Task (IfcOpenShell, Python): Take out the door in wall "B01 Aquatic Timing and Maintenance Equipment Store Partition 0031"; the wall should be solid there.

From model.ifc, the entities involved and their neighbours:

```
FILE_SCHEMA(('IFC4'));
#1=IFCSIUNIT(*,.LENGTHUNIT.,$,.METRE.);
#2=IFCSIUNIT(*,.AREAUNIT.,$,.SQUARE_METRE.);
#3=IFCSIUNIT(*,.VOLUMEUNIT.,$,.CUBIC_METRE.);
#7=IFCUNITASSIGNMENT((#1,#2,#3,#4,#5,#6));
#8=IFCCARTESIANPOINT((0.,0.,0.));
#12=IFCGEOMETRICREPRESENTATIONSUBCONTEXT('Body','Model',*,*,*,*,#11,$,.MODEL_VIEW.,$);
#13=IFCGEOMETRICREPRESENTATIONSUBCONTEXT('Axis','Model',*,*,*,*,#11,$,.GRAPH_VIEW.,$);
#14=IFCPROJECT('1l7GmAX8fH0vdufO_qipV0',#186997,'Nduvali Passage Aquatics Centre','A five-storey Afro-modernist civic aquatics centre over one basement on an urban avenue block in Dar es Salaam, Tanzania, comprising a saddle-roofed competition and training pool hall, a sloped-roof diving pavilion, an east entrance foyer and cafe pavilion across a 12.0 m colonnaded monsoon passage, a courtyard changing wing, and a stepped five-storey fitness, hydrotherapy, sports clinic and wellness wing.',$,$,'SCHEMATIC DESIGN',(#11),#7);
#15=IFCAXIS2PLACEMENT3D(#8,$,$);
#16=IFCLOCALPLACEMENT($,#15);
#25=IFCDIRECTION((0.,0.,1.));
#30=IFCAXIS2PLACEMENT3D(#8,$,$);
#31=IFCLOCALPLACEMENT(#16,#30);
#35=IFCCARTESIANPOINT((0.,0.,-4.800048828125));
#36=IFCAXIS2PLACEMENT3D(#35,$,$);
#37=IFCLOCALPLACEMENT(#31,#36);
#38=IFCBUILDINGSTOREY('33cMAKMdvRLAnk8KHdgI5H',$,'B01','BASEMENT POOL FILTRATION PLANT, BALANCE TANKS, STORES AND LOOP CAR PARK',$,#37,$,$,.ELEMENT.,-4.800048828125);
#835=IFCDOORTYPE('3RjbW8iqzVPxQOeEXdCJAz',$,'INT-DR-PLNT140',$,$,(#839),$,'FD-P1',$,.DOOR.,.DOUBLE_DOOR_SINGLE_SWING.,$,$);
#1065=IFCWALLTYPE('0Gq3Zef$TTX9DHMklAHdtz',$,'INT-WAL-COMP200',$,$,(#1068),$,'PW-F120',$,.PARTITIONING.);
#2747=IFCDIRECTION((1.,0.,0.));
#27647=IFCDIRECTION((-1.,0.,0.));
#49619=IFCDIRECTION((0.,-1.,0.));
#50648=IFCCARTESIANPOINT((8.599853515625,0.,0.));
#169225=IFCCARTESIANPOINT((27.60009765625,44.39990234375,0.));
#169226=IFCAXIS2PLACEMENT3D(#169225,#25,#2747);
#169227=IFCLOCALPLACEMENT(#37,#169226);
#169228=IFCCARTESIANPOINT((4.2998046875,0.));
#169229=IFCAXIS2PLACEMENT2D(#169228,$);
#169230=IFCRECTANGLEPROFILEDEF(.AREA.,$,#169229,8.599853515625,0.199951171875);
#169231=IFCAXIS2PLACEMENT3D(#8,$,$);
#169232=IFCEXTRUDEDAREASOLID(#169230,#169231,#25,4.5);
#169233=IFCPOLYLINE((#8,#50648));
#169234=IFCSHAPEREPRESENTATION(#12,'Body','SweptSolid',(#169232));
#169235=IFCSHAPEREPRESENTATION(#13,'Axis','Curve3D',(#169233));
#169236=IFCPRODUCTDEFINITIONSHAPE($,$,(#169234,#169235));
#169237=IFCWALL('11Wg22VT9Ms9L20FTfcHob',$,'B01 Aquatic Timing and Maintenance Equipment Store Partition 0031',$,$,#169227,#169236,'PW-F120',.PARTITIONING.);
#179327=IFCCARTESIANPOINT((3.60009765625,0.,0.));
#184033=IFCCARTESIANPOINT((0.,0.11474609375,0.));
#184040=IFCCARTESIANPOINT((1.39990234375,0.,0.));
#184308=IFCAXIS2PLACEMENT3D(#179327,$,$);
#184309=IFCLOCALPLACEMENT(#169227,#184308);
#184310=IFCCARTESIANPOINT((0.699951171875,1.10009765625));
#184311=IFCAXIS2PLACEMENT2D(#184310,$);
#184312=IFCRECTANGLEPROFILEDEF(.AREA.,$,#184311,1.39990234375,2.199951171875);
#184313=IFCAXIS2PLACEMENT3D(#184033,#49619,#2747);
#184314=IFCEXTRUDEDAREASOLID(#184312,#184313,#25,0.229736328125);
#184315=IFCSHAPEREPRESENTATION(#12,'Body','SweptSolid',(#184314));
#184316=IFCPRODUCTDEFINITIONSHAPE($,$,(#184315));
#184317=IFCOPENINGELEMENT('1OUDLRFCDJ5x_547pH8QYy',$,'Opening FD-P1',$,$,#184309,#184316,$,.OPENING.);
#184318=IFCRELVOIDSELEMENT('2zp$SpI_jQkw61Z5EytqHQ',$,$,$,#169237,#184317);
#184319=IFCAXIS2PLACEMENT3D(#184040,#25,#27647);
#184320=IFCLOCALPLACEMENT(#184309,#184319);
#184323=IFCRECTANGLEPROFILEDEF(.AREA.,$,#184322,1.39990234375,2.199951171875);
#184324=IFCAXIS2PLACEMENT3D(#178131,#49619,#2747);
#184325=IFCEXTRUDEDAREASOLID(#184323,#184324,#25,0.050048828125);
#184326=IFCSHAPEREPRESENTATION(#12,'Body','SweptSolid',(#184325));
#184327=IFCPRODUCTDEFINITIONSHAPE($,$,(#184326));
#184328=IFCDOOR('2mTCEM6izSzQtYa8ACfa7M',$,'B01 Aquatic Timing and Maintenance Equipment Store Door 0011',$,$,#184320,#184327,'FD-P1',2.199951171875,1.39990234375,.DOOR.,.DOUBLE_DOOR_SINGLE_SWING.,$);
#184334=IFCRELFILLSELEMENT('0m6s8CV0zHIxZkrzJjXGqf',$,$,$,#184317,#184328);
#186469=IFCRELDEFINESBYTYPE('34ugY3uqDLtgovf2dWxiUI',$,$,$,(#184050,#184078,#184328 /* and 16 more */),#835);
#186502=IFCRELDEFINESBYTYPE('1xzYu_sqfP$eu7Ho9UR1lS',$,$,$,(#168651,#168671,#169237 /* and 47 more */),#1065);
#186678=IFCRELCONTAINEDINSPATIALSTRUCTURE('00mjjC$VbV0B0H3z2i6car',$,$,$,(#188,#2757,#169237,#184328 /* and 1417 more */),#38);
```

```python
import ifcopenshell
import ifcopenshell.api.feature
import ifcopenshell.api.root
import ifcopenshell.geom
import ifcopenshell.util.shape

model = ifcopenshell.open("model.ifc")
settings = ifcopenshell.geom.settings()


def volume(element):
    """Net volume in cubic metres, openings subtracted."""
    shape = ifcopenshell.geom.create_shape(settings, element)
    return ifcopenshell.util.shape.get_volume(shape.geometry)


door = model.by_id(184328)
opening = door.FillsVoids[0].RelatingOpeningElement
wall = opening.VoidsElements[0].RelatingBuildingElement
before = volume(wall)

ifcopenshell.api.root.remove_product(model, product=door)
ifcopenshell.api.feature.remove_feature(model, feature=opening)

after = volume(wall)

print(f"wall volume {before:.3f} -> {after:.3f} m3")

model.write("model_v2.ifc")
```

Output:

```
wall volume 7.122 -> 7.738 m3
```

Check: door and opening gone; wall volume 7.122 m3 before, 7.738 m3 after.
